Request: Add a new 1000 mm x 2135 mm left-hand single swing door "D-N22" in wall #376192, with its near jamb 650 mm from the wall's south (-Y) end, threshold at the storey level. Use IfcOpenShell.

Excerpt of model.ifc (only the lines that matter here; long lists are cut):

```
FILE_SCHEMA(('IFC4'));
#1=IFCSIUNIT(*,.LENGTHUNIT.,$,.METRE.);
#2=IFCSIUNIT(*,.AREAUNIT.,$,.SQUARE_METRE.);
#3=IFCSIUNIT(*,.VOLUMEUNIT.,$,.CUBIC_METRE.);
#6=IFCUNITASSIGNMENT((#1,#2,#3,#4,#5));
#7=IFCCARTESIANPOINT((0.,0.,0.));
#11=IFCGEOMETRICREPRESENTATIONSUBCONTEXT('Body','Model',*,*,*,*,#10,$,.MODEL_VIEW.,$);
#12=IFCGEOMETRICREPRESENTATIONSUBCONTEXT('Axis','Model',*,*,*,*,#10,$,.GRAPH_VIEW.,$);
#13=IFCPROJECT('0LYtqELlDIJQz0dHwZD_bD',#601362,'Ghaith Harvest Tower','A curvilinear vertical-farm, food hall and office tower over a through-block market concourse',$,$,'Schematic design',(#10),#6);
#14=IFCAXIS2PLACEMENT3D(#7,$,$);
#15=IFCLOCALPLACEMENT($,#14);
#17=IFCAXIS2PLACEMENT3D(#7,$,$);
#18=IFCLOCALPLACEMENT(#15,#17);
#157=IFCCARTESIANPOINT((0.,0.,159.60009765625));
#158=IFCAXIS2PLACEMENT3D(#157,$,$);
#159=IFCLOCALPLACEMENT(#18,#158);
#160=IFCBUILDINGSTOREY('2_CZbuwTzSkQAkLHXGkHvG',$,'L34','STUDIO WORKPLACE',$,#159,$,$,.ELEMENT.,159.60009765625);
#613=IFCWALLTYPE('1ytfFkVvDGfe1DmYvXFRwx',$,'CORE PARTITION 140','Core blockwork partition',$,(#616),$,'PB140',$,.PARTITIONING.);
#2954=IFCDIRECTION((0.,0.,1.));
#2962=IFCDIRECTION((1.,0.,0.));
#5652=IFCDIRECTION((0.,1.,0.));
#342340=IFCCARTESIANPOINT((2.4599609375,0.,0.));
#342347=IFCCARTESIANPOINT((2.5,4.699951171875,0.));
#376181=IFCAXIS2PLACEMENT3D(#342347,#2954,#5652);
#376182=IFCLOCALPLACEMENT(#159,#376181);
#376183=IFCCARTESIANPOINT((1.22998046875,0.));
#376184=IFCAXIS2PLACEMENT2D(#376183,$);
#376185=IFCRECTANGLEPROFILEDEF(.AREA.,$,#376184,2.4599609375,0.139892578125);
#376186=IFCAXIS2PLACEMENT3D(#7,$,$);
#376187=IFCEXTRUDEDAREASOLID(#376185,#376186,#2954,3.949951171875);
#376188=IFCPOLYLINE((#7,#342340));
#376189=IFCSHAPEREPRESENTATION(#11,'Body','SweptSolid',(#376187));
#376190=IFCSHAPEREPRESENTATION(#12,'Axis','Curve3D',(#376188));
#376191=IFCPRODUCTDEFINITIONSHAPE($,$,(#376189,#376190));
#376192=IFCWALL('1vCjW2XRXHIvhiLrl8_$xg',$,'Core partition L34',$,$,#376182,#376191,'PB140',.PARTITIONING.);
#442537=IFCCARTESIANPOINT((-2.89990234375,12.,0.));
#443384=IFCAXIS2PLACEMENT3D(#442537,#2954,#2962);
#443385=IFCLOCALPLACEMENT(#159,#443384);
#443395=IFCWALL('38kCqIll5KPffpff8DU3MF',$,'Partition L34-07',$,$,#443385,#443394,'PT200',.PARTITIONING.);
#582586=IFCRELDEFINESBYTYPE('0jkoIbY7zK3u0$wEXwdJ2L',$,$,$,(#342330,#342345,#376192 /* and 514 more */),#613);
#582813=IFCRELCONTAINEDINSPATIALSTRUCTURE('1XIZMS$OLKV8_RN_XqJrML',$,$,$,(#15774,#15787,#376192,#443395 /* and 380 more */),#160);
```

```python
import numpy as np
import ifcopenshell
import ifcopenshell.api.feature
import ifcopenshell.api.geometry
import ifcopenshell.api.root
import ifcopenshell.api.spatial
import ifcopenshell.geom
import ifcopenshell.util.element
import ifcopenshell.util.placement
import ifcopenshell.util.representation
import ifcopenshell.util.shape
import ifcopenshell.util.unit

model = ifcopenshell.open("model.ifc")
unit_scale = ifcopenshell.util.unit.calculate_unit_scale(model)
settings = ifcopenshell.geom.settings()


def volume(element):
    """Net volume in cubic metres, openings subtracted."""
    shape = ifcopenshell.geom.create_shape(settings, element)
    return ifcopenshell.util.shape.get_volume(shape.geometry)


wall = model.by_id(376192)
storey = ifcopenshell.util.element.get_container(wall, ifc_class="IfcBuildingStorey")
context = ifcopenshell.util.representation.get_context(model, "Model", "Body", "MODEL_VIEW")
before = volume(wall)

width, height, from_end, sill = 1, 2.135, 0.65, 0.0  # metres

# The wall runs along its own X axis, and the end named is its -X end.
wall_shape = ifcopenshell.geom.create_shape(settings, wall)
x, y, z = ifcopenshell.util.shape.get_vertices(wall_shape.geometry).T
start = x.min() + from_end
face, thickness = float(y.min()), float(y.max() - y.min())
wall_matrix = ifcopenshell.util.placement.get_local_placement(wall.ObjectPlacement)
level = ifcopenshell.util.placement.get_local_placement(storey.ObjectPlacement)[2, 3]


def in_wall(x, y):
    """Placement at x, y metres in the wall's axes, at sill height."""
    matrix = wall_matrix.copy()
    matrix[:, 3] = wall_matrix @ np.array([x / unit_scale, y / unit_scale, 0.0, 1.0])
    matrix[2, 3] = level + sill / unit_scale
    return matrix


# Opening: a box that overshoots both wall faces by 50 mm.
opening = ifcopenshell.api.root.create_entity(model, ifc_class="IfcOpeningElement", predefined_type="OPENING")
box = ifcopenshell.api.geometry.add_wall_representation(
    model, context=context, length=width, height=height, thickness=thickness + 0.1
)
ifcopenshell.api.geometry.assign_representation(model, product=opening, representation=box)
ifcopenshell.api.geometry.edit_object_placement(model, product=opening, matrix=in_wall(start, face - 0.05), is_si=False)
ifcopenshell.api.feature.add_feature(model, feature=opening, element=wall)

door = ifcopenshell.api.root.create_entity(model, ifc_class="IfcDoor", name="D-N22", predefined_type="DOOR")
door.OverallWidth, door.OverallHeight = width / unit_scale, height / unit_scale
door.OperationType = "SINGLE_SWING_LEFT"
body = ifcopenshell.api.geometry.add_door_representation(
    model,
    context=context,
    overall_width=door.OverallWidth,
    overall_height=door.OverallHeight,
    operation_type="SINGLE_SWING_LEFT",
    lining_properties={"LiningDepth": thickness / unit_scale, "ThresholdDepth": thickness / unit_scale},
)
ifcopenshell.api.geometry.assign_representation(model, product=door, representation=body)
ifcopenshell.api.spatial.assign_container(model, products=[door], relating_structure=storey)
ifcopenshell.api.feature.add_filling(model, opening=opening, element=door)

# The lining spans the wall, so the door starts at the wall face.
ifcopenshell.api.geometry.edit_object_placement(model, product=door, matrix=in_wall(start, face), is_si=False)

after = volume(wall)

print(f"wall volume {before:.3f} -> {after:.3f} m3")

model.write("model_rev.ifc")
```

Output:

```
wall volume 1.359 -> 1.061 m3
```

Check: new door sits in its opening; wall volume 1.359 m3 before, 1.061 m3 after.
